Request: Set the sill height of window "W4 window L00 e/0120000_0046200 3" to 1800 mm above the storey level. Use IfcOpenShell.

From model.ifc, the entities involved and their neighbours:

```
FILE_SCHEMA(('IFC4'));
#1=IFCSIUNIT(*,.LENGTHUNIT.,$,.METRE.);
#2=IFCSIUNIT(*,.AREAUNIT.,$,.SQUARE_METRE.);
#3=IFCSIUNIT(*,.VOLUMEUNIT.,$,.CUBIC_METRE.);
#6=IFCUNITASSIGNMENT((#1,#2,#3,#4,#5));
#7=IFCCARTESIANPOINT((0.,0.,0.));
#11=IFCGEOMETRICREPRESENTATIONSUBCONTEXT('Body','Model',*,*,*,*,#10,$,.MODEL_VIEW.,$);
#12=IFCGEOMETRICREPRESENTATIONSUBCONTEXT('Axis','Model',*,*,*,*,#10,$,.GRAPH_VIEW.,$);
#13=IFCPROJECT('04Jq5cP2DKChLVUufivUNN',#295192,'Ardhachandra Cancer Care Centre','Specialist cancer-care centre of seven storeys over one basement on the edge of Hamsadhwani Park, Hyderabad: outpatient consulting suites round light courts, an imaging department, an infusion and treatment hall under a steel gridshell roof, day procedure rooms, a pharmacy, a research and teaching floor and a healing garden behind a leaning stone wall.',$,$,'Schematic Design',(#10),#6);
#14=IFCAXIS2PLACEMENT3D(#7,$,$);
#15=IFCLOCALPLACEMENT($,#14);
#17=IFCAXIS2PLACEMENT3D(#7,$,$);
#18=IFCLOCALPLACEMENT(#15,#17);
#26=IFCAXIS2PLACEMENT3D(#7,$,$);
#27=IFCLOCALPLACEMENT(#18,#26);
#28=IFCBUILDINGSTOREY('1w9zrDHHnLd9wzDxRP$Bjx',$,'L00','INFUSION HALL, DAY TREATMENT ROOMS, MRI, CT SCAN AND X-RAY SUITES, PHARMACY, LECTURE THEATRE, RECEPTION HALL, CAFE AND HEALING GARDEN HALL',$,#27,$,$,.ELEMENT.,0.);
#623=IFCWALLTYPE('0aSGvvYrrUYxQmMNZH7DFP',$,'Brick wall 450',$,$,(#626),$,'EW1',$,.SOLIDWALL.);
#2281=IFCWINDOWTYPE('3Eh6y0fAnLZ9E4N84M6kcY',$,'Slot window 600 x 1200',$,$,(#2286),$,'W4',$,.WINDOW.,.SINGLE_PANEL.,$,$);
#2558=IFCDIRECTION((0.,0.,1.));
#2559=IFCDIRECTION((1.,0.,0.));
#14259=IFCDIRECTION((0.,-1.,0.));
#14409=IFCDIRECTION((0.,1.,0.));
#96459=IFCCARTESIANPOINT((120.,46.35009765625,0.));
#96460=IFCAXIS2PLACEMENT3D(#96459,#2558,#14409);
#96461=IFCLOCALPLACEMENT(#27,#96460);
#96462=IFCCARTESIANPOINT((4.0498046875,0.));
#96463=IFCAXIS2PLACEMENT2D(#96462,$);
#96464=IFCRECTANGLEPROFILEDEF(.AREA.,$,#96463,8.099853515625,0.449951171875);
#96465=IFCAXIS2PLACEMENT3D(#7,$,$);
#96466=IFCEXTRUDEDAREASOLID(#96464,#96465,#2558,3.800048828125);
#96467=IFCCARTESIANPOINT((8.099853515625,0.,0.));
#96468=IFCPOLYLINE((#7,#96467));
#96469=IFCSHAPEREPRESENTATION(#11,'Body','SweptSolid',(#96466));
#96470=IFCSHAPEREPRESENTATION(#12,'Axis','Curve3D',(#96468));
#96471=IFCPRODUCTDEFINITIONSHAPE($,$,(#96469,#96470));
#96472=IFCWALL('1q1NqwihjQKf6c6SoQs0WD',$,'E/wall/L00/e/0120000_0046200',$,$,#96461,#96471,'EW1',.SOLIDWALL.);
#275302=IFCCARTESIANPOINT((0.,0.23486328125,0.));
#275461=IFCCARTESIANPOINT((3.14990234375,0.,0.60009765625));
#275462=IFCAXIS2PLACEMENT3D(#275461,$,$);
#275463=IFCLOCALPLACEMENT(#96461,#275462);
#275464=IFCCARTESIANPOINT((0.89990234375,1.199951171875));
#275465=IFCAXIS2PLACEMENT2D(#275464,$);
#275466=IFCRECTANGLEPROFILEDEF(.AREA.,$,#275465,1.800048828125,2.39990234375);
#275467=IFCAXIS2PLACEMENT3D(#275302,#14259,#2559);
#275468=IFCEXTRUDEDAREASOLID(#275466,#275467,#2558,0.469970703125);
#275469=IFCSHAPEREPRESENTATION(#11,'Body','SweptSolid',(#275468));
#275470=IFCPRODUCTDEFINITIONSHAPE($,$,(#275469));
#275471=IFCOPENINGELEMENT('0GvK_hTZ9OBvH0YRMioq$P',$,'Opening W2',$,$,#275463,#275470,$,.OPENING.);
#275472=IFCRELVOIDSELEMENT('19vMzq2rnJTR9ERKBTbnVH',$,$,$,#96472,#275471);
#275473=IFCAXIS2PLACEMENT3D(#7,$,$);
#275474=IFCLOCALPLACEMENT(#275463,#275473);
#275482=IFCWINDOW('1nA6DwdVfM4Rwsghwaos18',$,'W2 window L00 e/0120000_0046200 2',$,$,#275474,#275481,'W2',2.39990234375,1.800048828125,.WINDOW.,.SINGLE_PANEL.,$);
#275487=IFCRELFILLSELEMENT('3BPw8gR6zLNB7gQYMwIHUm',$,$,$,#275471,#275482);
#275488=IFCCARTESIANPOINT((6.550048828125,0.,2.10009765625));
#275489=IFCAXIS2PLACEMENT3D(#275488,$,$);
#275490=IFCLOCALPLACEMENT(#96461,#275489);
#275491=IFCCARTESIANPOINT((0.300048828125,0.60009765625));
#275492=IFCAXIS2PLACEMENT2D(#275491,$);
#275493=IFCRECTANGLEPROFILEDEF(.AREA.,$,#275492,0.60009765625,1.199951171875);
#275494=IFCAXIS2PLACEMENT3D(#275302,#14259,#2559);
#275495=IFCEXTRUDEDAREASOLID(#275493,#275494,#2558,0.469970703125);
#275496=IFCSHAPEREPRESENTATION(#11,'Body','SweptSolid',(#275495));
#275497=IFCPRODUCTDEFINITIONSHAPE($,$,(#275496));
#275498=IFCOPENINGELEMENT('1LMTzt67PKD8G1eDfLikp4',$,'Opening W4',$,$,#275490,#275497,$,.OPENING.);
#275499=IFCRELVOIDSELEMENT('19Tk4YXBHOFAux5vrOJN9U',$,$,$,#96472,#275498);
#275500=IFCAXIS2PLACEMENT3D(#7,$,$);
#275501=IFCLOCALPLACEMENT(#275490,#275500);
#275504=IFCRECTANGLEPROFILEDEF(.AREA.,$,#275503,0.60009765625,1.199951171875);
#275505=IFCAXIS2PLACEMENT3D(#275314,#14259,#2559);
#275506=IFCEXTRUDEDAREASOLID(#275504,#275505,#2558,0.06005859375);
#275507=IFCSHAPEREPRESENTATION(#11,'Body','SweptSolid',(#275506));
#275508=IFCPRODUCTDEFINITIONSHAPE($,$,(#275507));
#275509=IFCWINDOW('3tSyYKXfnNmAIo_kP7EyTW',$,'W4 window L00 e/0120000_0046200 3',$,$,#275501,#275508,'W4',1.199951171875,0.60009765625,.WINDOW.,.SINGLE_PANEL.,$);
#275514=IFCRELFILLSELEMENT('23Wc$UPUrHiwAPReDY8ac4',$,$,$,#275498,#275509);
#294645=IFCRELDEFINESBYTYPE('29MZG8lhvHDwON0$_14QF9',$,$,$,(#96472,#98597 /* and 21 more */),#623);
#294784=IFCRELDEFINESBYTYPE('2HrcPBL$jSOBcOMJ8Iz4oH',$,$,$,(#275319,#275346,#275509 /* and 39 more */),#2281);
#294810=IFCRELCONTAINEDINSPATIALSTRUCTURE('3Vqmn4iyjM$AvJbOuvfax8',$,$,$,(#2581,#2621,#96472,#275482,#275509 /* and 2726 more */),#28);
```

```python
import numpy as np
import ifcopenshell
import ifcopenshell.api.geometry
import ifcopenshell.geom
import ifcopenshell.util.element
import ifcopenshell.util.placement
import ifcopenshell.util.shape
import ifcopenshell.util.unit

model = ifcopenshell.open("model.ifc")
unit_scale = ifcopenshell.util.unit.calculate_unit_scale(model)

window = model.by_guid("3tSyYKXfnNmAIo_kP7EyTW")
opening = window.FillsVoids[0].RelatingOpeningElement
storey = ifcopenshell.util.element.get_container(window, ifc_class="IfcBuildingStorey")
level = ifcopenshell.util.placement.get_local_placement(storey.ObjectPlacement)[2, 3]

# The opening's origin need not be at the sill, so measure its lowest point.
shape = ifcopenshell.geom.create_shape(ifcopenshell.geom.settings(), opening)
bottom = ifcopenshell.util.shape.get_shape_bottom_elevation(shape, shape.geometry) / unit_scale
dz = level + 1.8 / unit_scale - bottom

shift = np.array([0.0, 0.0, dz])
# The window is placed relative to its opening, so it follows when the opening moves.
matrix = ifcopenshell.util.placement.get_local_placement(opening.ObjectPlacement)
matrix[:3, 3] += shift
ifcopenshell.api.geometry.edit_object_placement(
    model, product=opening, matrix=matrix, is_si=False, should_transform_children=True
)

print(f"moved by {dz * unit_scale:+.3f} m")

model.write("model_updated.ifc")
```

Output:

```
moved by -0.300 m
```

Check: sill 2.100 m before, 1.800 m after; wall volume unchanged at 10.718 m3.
